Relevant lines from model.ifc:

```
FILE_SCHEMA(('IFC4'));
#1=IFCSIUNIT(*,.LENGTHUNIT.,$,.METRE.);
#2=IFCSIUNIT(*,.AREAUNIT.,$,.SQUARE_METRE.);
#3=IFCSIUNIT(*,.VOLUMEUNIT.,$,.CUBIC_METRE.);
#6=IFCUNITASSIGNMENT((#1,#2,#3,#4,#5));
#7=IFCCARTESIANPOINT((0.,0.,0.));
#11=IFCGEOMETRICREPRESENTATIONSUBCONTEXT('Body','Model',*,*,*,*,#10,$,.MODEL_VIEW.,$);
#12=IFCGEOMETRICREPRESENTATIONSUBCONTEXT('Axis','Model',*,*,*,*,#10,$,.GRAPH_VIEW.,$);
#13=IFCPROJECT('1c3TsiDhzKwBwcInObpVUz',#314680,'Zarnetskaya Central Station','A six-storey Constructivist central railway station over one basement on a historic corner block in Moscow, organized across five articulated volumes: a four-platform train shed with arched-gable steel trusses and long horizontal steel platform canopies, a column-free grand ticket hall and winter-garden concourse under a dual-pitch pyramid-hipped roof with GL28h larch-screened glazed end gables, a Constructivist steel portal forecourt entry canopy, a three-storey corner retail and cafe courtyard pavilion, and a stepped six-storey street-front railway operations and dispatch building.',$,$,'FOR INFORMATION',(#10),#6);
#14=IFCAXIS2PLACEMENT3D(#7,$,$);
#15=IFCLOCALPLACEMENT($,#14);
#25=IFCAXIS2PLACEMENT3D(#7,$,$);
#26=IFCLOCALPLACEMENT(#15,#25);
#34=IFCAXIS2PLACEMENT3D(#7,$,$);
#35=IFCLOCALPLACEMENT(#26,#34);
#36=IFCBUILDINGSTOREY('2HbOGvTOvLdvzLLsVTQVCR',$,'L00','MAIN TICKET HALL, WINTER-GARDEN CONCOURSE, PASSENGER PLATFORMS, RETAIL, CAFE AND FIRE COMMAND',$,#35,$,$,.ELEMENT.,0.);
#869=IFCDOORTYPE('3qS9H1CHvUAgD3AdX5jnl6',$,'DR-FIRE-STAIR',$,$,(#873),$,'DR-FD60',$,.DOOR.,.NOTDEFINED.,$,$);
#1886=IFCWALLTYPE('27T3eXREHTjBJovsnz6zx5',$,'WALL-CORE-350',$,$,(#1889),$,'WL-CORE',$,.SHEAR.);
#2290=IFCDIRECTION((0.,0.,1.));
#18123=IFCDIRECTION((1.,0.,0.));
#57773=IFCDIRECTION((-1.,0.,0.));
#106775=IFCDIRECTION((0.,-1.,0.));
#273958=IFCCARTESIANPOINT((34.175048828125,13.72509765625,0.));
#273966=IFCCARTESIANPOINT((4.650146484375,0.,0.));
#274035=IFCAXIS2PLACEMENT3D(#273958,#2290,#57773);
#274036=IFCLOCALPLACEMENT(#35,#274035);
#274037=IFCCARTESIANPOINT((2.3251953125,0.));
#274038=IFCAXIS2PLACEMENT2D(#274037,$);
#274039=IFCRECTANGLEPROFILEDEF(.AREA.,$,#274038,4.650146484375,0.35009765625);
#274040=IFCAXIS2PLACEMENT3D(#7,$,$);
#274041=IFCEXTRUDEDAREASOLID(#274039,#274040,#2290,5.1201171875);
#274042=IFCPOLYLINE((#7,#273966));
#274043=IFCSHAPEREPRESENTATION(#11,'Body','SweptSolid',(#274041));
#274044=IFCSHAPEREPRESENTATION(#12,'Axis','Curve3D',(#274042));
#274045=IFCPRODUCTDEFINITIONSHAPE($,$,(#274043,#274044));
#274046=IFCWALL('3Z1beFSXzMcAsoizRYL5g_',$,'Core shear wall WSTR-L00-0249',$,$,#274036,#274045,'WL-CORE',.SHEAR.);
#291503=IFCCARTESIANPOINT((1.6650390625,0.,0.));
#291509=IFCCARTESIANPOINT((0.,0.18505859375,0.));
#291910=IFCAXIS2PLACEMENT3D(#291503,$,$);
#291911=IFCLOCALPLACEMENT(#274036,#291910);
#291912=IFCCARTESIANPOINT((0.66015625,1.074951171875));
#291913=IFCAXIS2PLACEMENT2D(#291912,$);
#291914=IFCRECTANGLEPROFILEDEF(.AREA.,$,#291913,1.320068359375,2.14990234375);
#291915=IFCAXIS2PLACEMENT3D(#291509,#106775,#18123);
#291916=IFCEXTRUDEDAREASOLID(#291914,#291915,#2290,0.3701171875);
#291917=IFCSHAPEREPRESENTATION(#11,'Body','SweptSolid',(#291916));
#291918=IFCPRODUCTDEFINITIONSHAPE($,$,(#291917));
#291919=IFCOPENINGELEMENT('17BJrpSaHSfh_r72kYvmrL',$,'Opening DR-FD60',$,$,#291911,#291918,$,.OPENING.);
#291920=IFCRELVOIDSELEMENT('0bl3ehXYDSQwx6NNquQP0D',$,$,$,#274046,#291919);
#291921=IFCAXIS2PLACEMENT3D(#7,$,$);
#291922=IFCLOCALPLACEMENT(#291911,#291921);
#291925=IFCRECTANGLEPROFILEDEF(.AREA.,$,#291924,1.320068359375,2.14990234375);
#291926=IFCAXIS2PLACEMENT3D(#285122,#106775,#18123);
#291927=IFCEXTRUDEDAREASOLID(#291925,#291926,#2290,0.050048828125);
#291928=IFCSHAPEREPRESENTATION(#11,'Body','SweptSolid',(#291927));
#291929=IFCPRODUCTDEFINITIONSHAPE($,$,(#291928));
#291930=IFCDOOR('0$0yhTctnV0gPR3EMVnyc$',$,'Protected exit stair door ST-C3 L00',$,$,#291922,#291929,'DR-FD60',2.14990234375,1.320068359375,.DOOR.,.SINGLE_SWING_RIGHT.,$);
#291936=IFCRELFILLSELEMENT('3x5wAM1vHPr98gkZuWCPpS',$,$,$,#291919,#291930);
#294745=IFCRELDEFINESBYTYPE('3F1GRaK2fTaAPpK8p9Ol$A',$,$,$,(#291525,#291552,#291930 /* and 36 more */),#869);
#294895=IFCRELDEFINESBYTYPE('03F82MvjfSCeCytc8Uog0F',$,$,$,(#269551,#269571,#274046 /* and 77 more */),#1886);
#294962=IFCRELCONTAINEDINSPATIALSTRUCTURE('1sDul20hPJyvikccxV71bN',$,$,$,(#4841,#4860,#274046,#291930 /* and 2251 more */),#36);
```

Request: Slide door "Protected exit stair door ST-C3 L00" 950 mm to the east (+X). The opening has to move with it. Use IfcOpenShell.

```python
import ifcopenshell
import ifcopenshell.api.geometry
import ifcopenshell.util.placement
import ifcopenshell.util.unit

model = ifcopenshell.open("model.ifc")
unit_scale = ifcopenshell.util.unit.calculate_unit_scale(model)

door = model.by_guid("0$0yhTctnV0gPR3EMVnyc$")
opening = door.FillsVoids[0].RelatingOpeningElement
wall = opening.VoidsElements[0].RelatingBuildingElement

wall_matrix = ifcopenshell.util.placement.get_local_placement(wall.ObjectPlacement)
shift = wall_matrix[:3, 0] * -0.95 / unit_scale
before = ifcopenshell.util.placement.get_local_placement(door.ObjectPlacement)[:3, 3].copy()

# The door is placed relative to its opening, so it follows when the opening moves.
matrix = ifcopenshell.util.placement.get_local_placement(opening.ObjectPlacement)
matrix[:3, 3] += shift
ifcopenshell.api.geometry.edit_object_placement(
    model, product=opening, matrix=matrix, is_si=False, should_transform_children=True
)

after = ifcopenshell.util.placement.get_local_placement(door.ObjectPlacement)[:3, 3]
print("door moved by", (after - before).round(3) + 0.0)

model.write("model_updated.ifc")
```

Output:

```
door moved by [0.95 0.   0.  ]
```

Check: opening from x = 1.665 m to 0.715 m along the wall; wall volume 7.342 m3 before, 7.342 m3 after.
